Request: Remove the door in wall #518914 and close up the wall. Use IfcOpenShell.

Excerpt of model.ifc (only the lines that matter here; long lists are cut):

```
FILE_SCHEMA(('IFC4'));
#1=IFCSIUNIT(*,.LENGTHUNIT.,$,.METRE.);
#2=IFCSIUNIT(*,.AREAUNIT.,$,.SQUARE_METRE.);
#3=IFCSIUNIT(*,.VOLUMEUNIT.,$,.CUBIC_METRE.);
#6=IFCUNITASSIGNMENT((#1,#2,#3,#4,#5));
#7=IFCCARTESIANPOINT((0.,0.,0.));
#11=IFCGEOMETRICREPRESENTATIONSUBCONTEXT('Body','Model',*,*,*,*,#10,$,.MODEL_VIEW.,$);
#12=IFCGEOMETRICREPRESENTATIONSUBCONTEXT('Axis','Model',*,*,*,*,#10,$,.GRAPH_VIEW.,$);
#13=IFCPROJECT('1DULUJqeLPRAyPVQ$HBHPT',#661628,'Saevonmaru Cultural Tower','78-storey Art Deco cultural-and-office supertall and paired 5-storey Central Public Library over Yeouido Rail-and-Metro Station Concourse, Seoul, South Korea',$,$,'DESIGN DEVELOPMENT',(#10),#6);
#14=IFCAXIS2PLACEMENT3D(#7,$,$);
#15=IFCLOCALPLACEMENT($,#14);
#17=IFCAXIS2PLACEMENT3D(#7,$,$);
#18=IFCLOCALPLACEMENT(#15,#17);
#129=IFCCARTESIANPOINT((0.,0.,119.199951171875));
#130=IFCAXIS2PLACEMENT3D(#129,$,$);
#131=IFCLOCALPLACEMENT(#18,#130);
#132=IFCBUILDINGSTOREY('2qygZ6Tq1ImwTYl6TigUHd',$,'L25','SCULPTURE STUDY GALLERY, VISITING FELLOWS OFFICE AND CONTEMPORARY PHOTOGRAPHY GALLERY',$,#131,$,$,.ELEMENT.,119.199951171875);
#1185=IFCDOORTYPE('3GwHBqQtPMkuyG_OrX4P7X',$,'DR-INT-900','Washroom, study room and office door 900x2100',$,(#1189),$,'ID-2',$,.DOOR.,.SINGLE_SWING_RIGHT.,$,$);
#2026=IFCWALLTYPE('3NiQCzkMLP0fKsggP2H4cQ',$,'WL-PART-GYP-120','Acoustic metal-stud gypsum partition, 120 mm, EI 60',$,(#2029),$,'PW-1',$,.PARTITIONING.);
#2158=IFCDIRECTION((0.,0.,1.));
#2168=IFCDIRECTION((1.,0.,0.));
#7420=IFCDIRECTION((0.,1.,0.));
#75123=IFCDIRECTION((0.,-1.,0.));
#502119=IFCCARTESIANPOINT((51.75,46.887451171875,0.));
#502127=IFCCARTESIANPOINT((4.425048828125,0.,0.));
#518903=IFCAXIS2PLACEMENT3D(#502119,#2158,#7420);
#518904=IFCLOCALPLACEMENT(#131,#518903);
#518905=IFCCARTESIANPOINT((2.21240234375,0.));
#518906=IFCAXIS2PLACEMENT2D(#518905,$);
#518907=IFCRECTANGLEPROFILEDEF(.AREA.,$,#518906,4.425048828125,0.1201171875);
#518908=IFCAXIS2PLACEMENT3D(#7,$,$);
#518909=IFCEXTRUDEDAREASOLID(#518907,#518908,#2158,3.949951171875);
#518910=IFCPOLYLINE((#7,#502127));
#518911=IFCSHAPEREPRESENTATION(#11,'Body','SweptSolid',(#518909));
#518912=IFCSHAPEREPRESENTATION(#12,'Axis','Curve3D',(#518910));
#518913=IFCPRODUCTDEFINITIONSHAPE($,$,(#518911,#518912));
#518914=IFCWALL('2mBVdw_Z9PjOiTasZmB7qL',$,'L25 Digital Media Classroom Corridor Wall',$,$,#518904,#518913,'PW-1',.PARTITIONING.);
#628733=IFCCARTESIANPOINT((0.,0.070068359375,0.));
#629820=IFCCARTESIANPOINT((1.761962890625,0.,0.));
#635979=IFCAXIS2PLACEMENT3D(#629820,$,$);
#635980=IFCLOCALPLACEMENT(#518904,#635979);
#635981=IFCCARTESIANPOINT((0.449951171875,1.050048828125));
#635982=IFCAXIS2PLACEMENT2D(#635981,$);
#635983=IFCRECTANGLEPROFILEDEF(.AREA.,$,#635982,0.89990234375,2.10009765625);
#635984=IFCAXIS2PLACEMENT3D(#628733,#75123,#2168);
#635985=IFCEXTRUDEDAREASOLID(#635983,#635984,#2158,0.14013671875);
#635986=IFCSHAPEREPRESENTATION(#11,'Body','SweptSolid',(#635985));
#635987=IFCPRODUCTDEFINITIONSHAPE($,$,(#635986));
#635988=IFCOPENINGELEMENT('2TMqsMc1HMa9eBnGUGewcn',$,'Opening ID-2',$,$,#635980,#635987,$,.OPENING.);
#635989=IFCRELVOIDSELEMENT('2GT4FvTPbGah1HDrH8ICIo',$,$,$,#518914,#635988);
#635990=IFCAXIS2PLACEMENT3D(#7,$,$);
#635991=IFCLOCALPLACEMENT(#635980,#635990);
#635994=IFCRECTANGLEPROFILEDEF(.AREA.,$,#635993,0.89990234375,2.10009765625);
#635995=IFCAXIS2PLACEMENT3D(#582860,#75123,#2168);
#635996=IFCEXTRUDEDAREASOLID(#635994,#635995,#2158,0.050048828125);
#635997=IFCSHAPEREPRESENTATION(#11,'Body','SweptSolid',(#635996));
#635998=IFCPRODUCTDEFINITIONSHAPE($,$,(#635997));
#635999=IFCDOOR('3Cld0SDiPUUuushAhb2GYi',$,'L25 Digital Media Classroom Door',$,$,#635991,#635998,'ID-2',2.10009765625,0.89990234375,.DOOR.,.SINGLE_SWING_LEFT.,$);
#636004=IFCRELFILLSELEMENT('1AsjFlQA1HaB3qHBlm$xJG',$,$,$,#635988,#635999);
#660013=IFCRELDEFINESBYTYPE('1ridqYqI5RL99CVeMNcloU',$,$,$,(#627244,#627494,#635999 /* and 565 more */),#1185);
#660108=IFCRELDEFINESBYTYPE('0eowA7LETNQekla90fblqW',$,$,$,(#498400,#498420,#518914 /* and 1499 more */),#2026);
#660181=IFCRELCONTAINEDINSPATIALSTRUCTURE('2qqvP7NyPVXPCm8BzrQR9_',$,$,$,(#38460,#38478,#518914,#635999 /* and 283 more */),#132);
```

```python
import ifcopenshell
import ifcopenshell.api.feature
import ifcopenshell.api.root
import ifcopenshell.geom
import ifcopenshell.util.shape

model = ifcopenshell.open("model.ifc")
settings = ifcopenshell.geom.settings()


def volume(element):
    """Net volume in cubic metres, openings subtracted."""
    shape = ifcopenshell.geom.create_shape(settings, element)
    return ifcopenshell.util.shape.get_volume(shape.geometry)


door = model.by_guid("3Cld0SDiPUUuushAhb2GYi")
opening = door.FillsVoids[0].RelatingOpeningElement
wall = opening.VoidsElements[0].RelatingBuildingElement
before = volume(wall)

ifcopenshell.api.root.remove_product(model, product=door)
ifcopenshell.api.feature.remove_feature(model, feature=opening)

after = volume(wall)

print(f"wall volume {before:.3f} -> {after:.3f} m3")

model.write("model_edited.ifc")
```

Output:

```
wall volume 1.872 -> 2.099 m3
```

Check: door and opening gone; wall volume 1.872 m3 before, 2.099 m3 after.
